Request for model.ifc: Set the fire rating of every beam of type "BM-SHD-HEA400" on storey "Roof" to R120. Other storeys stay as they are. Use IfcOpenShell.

First a look at what the model holds.

```python
import ifcopenshell
import ifcopenshell.util.element

model = ifcopenshell.open("model.ifc")
print(model.schema)
storey = next(s for s in model.by_type("IfcBuildingStorey") if s.Name == "Roof")
beams = [e for e in ifcopenshell.util.element.get_decomposition(storey) if e.is_a("IfcBeam")]
seen = {}
for e in beams:
    element_type = ifcopenshell.util.element.get_type(e)
    key = (element_type.Name if element_type != e and element_type else None, ifcopenshell.util.element.get_pset(e, "Pset_BeamCommon", "FireRating"))
    seen[key] = seen.get(key, 0) + 1
for (name, value), count in sorted(seen.items(), key=str):
    print(count, "x", name, "|", value)
```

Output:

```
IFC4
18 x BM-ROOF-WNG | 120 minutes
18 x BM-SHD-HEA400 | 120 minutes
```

```python
import ifcopenshell
import ifcopenshell.api.pset
import ifcopenshell.util.element

model = ifcopenshell.open("model.ifc")

storey = next(s for s in model.by_type("IfcBuildingStorey") if s.Name == "Roof")
beams = [e for e in ifcopenshell.util.element.get_decomposition(storey) if e.is_a("IfcBeam")]

count = 0
for e in beams:
    element_type = ifcopenshell.util.element.get_type(e)
    if element_type in (None, e) or element_type.Name != "BM-SHD-HEA400":
        continue
    # add_pset returns the element's existing set when there is one.
    pset = ifcopenshell.api.pset.add_pset(model, product=e, name="Pset_BeamCommon")
    ifcopenshell.api.pset.edit_pset(model, pset=pset, properties={"FireRating": "R120"})
    count += 1

print(count, "beams updated")

model.write("model_edited.ifc")
```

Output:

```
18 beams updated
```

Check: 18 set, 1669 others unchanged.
